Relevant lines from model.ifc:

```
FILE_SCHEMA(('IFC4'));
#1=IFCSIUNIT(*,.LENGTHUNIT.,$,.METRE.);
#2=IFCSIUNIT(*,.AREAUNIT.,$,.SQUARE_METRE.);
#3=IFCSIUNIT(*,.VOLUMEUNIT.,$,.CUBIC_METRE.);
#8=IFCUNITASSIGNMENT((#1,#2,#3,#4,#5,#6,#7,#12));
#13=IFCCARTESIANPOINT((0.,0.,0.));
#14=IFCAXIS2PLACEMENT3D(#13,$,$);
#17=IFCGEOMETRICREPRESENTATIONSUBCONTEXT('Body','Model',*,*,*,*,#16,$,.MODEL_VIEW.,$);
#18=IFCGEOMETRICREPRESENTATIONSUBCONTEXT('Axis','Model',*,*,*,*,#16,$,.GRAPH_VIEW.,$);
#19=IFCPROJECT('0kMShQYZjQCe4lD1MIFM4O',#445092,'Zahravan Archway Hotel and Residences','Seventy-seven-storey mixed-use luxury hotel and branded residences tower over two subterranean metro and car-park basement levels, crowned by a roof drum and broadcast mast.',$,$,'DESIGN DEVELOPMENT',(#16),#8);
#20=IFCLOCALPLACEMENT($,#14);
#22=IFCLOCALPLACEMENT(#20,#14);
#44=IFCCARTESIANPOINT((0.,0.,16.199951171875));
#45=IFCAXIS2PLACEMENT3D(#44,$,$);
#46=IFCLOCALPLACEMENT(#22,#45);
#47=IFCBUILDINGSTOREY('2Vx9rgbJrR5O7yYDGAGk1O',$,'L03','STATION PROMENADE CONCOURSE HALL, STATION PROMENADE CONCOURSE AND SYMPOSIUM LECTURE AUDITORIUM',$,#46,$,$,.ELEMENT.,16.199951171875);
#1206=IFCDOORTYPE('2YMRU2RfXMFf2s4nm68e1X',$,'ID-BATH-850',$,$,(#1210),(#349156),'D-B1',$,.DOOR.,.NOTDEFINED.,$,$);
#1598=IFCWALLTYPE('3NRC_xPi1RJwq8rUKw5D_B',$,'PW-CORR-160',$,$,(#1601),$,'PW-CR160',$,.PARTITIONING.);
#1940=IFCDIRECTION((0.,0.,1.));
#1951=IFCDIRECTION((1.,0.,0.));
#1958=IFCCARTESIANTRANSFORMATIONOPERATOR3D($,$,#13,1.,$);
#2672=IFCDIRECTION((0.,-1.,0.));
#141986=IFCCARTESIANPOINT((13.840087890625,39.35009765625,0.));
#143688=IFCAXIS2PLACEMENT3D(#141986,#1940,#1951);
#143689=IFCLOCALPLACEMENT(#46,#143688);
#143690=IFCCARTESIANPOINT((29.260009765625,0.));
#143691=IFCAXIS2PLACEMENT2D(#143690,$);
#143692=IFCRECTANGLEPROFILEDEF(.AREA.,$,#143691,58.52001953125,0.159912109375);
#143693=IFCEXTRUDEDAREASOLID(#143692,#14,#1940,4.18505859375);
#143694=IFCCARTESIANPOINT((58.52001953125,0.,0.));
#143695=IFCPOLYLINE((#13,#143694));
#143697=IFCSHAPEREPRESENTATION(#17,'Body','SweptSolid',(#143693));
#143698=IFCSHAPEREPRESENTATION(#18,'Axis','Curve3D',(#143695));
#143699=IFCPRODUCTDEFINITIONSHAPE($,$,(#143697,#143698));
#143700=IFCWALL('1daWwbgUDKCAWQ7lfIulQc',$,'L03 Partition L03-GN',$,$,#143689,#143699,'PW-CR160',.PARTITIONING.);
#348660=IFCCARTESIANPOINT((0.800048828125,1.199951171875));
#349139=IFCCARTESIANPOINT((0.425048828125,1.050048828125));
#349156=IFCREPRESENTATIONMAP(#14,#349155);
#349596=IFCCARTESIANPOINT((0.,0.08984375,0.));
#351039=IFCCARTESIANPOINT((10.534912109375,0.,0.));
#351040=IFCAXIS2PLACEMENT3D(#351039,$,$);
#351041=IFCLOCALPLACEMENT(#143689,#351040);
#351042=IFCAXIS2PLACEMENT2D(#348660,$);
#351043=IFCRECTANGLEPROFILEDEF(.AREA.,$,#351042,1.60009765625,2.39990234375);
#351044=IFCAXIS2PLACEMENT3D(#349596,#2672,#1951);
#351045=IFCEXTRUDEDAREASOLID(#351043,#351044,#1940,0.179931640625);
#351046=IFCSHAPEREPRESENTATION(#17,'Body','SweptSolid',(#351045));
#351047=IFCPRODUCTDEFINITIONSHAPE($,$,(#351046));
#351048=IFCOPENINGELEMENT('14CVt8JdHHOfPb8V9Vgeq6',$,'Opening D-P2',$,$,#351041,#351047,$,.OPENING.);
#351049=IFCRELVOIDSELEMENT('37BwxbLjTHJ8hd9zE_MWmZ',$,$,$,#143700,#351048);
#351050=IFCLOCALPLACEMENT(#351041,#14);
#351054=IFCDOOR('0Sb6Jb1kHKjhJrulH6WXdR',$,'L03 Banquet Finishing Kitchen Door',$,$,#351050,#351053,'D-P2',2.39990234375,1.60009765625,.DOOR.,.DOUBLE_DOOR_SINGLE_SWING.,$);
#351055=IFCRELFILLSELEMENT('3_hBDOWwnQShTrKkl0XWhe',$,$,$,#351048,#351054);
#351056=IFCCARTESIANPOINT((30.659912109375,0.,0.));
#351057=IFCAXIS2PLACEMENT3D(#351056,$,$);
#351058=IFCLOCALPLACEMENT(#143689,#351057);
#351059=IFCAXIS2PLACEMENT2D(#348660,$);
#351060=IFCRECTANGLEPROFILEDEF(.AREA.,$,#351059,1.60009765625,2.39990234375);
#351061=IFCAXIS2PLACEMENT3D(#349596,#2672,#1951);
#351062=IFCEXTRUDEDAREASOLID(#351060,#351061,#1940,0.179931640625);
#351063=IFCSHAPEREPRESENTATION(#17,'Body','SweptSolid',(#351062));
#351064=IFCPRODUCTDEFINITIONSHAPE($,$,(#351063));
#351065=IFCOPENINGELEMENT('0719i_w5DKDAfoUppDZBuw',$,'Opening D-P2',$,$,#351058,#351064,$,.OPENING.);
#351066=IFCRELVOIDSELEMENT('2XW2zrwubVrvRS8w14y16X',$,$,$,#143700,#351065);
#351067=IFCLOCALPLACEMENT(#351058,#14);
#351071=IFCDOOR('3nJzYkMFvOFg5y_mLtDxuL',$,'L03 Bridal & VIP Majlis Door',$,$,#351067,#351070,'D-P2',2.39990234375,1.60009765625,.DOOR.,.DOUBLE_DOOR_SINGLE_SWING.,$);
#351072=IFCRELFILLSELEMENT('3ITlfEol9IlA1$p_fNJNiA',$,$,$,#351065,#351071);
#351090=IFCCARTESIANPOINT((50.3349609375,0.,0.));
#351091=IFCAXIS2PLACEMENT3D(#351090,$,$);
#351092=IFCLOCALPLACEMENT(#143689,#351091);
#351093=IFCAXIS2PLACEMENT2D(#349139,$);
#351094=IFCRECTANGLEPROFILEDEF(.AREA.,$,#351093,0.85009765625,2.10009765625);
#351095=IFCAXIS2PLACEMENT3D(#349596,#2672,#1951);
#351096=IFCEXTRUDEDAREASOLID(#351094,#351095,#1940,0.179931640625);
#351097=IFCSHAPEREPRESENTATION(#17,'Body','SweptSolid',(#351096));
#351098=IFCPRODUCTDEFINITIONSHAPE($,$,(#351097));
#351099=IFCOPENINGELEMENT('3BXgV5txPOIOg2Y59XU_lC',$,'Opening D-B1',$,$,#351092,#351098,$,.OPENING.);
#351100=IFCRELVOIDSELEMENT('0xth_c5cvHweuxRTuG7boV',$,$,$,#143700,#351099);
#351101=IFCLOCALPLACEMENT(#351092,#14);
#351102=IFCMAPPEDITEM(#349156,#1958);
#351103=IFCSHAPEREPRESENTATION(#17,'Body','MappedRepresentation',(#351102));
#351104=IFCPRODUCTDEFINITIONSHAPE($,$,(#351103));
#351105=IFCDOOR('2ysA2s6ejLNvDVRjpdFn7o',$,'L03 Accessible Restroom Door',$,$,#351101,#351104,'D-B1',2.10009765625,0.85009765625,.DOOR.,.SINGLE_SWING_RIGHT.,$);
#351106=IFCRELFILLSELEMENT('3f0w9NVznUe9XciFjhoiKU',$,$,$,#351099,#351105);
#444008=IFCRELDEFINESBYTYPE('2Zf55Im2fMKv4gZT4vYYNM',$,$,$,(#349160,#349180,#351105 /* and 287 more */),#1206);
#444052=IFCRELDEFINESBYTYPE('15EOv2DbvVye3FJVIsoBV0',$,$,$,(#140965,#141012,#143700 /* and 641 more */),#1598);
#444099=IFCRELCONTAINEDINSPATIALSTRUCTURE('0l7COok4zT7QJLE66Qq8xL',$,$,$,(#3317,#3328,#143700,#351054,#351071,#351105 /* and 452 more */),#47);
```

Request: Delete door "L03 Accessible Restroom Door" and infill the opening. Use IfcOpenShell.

```python
import ifcopenshell
import ifcopenshell.api.feature
import ifcopenshell.api.root
import ifcopenshell.geom
import ifcopenshell.util.shape

model = ifcopenshell.open("model.ifc")
settings = ifcopenshell.geom.settings()


def volume(element):
    """Net volume in cubic metres, openings subtracted."""
    shape = ifcopenshell.geom.create_shape(settings, element)
    return ifcopenshell.util.shape.get_volume(shape.geometry)


door = model.by_id(351105)
opening = door.FillsVoids[0].RelatingOpeningElement
wall = opening.VoidsElements[0].RelatingBuildingElement
before = volume(wall)

ifcopenshell.api.root.remove_product(model, product=door)
ifcopenshell.api.feature.remove_feature(model, feature=opening)

after = volume(wall)

print(f"wall volume {before:.3f} -> {after:.3f} m3")

model.write("model_v2.ifc")
```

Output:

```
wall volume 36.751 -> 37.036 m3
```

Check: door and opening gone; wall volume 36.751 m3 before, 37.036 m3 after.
